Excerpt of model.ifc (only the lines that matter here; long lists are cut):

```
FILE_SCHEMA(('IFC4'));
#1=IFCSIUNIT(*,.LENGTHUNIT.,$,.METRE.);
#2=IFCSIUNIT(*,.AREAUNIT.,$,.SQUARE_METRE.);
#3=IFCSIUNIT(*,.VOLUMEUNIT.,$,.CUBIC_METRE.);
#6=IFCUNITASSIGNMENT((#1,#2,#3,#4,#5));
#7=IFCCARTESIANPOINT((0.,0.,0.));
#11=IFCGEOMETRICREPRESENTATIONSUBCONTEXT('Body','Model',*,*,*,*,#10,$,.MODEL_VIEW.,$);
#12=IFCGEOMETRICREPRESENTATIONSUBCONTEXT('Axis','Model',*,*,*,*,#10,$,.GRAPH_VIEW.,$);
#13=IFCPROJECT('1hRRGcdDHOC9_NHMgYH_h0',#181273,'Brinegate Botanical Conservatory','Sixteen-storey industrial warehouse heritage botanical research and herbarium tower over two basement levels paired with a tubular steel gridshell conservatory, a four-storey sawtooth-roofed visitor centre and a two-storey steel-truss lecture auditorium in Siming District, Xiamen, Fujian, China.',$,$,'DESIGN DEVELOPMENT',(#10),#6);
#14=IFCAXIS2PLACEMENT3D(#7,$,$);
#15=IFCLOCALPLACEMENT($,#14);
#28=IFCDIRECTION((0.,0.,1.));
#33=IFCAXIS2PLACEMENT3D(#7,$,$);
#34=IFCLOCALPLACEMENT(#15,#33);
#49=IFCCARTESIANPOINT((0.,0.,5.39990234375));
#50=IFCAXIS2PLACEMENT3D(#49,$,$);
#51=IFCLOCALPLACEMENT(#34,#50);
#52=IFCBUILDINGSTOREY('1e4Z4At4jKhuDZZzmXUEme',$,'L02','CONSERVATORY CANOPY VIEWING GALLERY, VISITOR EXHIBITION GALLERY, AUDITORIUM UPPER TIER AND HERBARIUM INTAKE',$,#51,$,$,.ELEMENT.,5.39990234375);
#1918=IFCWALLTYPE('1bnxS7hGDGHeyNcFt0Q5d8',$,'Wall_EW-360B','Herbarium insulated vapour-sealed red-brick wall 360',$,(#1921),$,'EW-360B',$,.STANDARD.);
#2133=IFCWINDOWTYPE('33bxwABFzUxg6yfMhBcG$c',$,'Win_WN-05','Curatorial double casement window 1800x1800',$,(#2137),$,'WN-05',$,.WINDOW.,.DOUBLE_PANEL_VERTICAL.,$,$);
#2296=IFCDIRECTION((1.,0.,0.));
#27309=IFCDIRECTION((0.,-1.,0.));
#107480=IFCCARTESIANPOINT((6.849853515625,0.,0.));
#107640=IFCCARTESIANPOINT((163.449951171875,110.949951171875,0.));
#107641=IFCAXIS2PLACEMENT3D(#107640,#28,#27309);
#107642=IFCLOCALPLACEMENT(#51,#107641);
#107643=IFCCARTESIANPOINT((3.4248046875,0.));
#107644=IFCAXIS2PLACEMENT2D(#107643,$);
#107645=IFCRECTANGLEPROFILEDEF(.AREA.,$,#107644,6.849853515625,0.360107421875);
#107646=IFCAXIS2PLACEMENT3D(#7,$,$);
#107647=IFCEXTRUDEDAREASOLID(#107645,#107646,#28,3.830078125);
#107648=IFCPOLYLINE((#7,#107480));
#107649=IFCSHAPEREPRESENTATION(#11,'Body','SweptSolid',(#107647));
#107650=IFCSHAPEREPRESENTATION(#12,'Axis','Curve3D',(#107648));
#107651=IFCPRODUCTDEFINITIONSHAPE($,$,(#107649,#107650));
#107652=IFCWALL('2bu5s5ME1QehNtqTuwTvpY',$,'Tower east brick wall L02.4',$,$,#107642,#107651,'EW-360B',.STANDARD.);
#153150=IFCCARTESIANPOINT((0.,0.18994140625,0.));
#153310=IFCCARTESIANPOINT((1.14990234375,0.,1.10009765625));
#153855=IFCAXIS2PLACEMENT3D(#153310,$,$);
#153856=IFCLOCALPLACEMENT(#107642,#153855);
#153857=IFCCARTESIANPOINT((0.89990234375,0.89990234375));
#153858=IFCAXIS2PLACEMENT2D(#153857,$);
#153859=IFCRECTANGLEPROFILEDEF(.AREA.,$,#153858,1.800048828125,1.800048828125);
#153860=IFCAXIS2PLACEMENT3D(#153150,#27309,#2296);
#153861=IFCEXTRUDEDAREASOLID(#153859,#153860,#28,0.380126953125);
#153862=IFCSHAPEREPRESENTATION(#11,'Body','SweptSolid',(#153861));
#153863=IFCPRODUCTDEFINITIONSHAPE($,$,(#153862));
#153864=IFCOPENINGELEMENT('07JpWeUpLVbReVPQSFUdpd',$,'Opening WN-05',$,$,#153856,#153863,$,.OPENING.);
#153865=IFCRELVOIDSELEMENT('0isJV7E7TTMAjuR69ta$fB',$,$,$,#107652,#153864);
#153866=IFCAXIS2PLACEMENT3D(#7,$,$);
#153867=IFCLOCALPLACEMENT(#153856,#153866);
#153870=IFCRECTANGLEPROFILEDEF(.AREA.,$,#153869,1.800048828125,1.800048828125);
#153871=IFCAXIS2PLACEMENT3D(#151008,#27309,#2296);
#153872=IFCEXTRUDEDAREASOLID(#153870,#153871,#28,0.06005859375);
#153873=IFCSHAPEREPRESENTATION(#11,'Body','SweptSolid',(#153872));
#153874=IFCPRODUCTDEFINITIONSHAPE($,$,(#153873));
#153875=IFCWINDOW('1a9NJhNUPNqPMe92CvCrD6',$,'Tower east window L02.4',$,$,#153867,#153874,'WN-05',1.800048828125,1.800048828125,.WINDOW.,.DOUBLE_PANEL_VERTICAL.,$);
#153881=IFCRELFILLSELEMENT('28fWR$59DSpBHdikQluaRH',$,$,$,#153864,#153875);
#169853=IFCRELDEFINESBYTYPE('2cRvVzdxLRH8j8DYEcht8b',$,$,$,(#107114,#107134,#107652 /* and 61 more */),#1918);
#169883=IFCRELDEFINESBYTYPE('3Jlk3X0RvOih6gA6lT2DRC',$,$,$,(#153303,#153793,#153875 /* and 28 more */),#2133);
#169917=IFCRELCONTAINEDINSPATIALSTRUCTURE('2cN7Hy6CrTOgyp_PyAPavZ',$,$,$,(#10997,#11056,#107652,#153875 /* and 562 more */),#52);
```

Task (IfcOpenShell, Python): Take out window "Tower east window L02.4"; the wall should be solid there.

```python
import ifcopenshell
import ifcopenshell.api.feature
import ifcopenshell.api.root
import ifcopenshell.geom
import ifcopenshell.util.shape

model = ifcopenshell.open("model.ifc")
settings = ifcopenshell.geom.settings()


def volume(element):
    """Net volume in cubic metres, openings subtracted."""
    shape = ifcopenshell.geom.create_shape(settings, element)
    return ifcopenshell.util.shape.get_volume(shape.geometry)


window = model.by_guid("1a9NJhNUPNqPMe92CvCrD6")
opening = window.FillsVoids[0].RelatingOpeningElement
wall = opening.VoidsElements[0].RelatingBuildingElement
before = volume(wall)

ifcopenshell.api.root.remove_product(model, product=window)
ifcopenshell.api.feature.remove_feature(model, feature=opening)

after = volume(wall)

print(f"wall volume {before:.3f} -> {after:.3f} m3")

model.write("model_updated.ifc")
```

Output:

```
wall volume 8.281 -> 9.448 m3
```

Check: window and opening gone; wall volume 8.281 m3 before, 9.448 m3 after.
